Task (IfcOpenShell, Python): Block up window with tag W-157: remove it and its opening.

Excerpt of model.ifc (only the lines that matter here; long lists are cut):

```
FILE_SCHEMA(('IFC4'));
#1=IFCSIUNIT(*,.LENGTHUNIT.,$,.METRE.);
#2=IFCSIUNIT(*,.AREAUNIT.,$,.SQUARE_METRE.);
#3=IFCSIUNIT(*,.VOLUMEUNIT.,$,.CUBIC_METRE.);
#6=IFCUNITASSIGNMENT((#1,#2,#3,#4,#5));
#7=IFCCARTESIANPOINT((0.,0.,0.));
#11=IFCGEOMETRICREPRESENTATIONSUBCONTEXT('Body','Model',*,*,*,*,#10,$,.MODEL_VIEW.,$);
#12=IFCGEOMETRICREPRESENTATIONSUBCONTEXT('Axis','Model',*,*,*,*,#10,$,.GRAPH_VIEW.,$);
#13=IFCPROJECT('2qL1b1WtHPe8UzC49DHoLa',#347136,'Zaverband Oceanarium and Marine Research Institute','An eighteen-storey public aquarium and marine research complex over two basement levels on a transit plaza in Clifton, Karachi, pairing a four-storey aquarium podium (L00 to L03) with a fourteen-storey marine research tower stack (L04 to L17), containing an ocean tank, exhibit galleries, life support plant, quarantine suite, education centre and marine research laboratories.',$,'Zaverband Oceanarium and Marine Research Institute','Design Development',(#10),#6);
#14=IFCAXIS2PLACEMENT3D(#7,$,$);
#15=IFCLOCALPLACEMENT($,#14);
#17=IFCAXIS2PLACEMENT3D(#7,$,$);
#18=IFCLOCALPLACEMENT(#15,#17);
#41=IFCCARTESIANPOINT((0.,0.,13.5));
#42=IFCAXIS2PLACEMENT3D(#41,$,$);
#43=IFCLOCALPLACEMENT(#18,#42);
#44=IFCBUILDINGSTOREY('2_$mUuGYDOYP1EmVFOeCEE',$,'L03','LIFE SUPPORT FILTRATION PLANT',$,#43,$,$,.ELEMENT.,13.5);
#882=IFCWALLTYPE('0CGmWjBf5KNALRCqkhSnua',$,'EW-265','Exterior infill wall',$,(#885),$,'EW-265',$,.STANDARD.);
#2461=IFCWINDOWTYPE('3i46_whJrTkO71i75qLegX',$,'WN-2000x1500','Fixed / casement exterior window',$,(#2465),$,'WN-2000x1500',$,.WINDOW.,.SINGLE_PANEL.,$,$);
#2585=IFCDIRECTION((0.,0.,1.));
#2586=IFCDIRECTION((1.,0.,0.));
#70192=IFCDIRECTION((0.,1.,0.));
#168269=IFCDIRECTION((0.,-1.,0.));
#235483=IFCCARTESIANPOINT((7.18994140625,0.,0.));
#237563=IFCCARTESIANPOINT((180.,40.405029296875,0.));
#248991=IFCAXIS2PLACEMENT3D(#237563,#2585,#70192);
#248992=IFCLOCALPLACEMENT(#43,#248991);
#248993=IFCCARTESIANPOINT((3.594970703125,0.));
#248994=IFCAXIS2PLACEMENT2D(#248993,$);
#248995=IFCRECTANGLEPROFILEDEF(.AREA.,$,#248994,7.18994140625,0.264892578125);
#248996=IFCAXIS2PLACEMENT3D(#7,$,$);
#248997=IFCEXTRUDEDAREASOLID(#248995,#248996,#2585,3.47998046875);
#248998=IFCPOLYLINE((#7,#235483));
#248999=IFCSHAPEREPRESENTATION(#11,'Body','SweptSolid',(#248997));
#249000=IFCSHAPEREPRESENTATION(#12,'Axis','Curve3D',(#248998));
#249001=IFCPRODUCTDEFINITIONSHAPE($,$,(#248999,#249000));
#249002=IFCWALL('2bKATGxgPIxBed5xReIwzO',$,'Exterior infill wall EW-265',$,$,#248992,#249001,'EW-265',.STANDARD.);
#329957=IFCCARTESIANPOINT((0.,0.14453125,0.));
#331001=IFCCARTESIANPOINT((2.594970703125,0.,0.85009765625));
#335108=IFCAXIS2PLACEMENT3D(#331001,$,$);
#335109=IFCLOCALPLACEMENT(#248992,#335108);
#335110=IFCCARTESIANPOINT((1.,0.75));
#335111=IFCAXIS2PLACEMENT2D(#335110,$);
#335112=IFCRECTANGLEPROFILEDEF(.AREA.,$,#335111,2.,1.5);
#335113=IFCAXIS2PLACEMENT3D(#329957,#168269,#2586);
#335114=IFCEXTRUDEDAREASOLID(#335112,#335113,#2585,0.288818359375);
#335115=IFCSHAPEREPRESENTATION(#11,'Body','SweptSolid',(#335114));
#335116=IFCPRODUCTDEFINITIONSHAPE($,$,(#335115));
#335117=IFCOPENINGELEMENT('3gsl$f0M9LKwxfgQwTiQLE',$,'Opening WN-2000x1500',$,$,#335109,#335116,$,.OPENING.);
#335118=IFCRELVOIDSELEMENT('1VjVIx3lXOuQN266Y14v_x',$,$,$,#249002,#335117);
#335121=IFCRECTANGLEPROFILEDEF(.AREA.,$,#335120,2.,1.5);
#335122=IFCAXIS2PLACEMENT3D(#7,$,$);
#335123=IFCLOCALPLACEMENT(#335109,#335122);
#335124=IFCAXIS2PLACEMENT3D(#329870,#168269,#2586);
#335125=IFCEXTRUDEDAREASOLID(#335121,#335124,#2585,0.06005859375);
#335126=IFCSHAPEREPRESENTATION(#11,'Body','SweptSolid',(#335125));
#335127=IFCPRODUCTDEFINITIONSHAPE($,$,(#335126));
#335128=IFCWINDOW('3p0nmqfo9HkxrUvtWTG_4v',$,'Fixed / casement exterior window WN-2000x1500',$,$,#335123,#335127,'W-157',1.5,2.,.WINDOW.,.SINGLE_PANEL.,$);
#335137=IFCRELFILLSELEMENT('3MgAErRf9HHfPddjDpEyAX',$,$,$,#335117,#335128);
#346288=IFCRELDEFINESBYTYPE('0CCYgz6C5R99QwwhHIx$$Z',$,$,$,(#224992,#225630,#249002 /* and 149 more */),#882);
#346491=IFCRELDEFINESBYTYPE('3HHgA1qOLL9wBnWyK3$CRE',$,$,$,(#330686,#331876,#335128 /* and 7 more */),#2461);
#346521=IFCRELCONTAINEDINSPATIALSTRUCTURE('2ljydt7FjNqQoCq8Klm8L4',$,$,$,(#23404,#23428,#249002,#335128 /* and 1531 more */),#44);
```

```python
import ifcopenshell
import ifcopenshell.api.feature
import ifcopenshell.api.root
import ifcopenshell.geom
import ifcopenshell.util.shape

model = ifcopenshell.open("model.ifc")
settings = ifcopenshell.geom.settings()


def volume(element):
    """Net volume in cubic metres, openings subtracted."""
    shape = ifcopenshell.geom.create_shape(settings, element)
    return ifcopenshell.util.shape.get_volume(shape.geometry)


window = model.by_guid("3p0nmqfo9HkxrUvtWTG_4v")
opening = window.FillsVoids[0].RelatingOpeningElement
wall = opening.VoidsElements[0].RelatingBuildingElement
before = volume(wall)

ifcopenshell.api.root.remove_product(model, product=window)
ifcopenshell.api.feature.remove_feature(model, feature=opening)

after = volume(wall)

print(f"wall volume {before:.3f} -> {after:.3f} m3")

model.write("model_rev.ifc")
```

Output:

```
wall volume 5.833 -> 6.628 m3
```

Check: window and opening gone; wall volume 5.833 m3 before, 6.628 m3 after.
